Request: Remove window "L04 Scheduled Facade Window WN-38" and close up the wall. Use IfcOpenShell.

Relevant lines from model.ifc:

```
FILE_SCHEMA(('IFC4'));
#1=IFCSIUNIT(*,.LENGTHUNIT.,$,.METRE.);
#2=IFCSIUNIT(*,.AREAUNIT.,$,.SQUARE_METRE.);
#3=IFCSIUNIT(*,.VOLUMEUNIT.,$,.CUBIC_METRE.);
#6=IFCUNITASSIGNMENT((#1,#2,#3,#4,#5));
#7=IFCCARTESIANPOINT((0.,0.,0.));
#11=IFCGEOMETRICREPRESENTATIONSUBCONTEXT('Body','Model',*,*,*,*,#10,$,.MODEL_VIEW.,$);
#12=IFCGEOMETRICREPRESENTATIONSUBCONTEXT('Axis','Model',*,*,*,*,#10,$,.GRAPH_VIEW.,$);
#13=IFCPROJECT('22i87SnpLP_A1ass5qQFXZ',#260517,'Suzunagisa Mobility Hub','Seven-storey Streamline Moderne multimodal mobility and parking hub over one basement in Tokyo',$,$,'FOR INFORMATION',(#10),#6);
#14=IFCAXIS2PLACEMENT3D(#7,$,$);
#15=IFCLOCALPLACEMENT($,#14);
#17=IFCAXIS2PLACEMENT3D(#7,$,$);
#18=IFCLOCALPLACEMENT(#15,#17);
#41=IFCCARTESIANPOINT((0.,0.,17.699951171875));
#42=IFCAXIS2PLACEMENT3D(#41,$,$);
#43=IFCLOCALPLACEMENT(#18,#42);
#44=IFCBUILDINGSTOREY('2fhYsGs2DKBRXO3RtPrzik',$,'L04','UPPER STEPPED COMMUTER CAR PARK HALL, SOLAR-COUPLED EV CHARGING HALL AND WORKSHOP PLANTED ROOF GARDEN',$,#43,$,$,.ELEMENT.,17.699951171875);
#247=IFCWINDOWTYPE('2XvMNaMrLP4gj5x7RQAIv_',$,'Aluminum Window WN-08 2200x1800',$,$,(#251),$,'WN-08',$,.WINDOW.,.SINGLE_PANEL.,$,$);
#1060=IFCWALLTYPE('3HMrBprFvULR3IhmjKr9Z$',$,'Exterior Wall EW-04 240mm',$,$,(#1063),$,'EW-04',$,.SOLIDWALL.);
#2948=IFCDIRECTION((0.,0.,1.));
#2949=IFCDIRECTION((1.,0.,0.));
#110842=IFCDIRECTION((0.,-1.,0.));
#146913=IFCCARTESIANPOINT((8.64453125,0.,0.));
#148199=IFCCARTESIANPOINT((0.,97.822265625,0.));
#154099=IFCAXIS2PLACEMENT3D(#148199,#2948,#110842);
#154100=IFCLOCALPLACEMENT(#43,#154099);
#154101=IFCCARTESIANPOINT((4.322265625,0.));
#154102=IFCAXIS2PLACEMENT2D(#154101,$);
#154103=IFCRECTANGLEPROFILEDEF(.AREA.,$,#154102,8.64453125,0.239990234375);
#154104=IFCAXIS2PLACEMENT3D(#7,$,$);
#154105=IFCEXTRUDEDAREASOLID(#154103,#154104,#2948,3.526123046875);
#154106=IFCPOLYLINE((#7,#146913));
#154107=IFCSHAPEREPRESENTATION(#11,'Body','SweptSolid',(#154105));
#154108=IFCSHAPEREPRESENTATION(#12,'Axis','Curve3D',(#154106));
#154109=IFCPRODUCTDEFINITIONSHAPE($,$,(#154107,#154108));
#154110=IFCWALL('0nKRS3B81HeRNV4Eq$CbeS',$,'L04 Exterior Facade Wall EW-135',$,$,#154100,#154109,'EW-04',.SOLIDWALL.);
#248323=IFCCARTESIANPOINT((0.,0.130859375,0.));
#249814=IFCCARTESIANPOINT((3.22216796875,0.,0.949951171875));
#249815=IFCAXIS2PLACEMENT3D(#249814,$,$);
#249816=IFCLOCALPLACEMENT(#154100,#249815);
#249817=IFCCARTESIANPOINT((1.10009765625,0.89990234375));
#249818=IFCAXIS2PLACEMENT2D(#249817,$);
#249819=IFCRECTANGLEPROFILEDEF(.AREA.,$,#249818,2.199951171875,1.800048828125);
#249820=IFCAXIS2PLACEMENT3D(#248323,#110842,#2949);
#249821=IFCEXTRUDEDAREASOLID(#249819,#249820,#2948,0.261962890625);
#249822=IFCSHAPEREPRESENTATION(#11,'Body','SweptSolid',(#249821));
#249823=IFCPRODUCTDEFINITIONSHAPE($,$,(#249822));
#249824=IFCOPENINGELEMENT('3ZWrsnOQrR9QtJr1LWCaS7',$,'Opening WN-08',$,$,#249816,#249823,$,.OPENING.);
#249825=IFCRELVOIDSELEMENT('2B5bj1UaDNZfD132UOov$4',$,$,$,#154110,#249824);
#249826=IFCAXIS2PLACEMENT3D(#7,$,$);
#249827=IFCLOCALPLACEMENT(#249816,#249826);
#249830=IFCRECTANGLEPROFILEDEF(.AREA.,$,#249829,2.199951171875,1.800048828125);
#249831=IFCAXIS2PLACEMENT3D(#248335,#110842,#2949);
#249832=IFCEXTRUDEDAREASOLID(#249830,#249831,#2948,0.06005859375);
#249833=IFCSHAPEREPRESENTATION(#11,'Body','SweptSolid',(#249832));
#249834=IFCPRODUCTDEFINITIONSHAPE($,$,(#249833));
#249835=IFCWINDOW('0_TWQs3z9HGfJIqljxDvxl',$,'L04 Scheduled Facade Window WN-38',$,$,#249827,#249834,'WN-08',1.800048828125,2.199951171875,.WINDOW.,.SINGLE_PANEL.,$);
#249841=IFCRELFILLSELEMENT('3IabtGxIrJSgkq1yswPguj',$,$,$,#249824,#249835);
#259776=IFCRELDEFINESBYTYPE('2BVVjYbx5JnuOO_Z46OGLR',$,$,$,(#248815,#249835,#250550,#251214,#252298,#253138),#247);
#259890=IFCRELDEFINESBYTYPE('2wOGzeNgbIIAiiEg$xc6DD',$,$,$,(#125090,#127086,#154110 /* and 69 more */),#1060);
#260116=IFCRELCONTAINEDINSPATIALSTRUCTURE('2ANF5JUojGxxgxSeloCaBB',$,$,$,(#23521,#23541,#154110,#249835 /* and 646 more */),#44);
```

```python
import ifcopenshell
import ifcopenshell.api.feature
import ifcopenshell.api.root
import ifcopenshell.geom
import ifcopenshell.util.shape

model = ifcopenshell.open("model.ifc")
settings = ifcopenshell.geom.settings()


def volume(element):
    """Net volume in cubic metres, openings subtracted."""
    shape = ifcopenshell.geom.create_shape(settings, element)
    return ifcopenshell.util.shape.get_volume(shape.geometry)


window = model.by_id(249835)
opening = window.FillsVoids[0].RelatingOpeningElement
wall = opening.VoidsElements[0].RelatingBuildingElement
before = volume(wall)

ifcopenshell.api.root.remove_product(model, product=window)
ifcopenshell.api.feature.remove_feature(model, feature=opening)

after = volume(wall)

print(f"wall volume {before:.3f} -> {after:.3f} m3")

model.write("model_rev.ifc")
```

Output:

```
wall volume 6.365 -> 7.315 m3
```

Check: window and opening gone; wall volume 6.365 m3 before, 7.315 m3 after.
